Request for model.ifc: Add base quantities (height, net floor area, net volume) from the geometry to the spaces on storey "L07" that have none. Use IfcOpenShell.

First a look at what the model holds.

```python
import ifcopenshell
import ifcopenshell.util.element
import ifcopenshell.util.unit

model = ifcopenshell.open("model.ifc")
print(model.schema)
for unit_type in ("LENGTHUNIT", "AREAUNIT", "VOLUMEUNIT"):
    print(unit_type, ifcopenshell.util.unit.calculate_unit_scale(model, unit_type))
storey = next(s for s in model.by_type("IfcBuildingStorey") if s.Name == "L07")
spaces = [e for e in ifcopenshell.util.element.get_decomposition(storey) if e.is_a("IfcSpace")]
for e in sorted(spaces, key=lambda e: e.id()):
    print(e.id(), e.is_a(), e.Name, list(ifcopenshell.util.element.get_psets(e, qtos_only=True)), sep=" | ")
```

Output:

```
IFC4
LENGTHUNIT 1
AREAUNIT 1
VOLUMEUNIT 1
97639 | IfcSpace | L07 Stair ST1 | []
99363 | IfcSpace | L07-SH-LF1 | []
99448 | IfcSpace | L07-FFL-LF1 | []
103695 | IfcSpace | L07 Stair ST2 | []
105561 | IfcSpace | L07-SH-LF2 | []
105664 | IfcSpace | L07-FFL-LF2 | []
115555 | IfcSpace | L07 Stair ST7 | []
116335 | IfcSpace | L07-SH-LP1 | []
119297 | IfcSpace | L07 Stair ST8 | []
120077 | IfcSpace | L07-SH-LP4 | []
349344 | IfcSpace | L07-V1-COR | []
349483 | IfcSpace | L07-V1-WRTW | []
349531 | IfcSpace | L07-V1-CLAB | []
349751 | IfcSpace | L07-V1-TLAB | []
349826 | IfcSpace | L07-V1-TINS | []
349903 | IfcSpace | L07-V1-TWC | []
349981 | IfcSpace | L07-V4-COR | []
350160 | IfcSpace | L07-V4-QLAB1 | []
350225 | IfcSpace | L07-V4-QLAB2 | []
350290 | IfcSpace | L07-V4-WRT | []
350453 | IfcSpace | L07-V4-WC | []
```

```python
import ifcopenshell
import ifcopenshell.api.pset
import ifcopenshell.geom
import ifcopenshell.util.element
import ifcopenshell.util.shape
import ifcopenshell.util.unit

model = ifcopenshell.open("model.ifc")
unit_scale = ifcopenshell.util.unit.calculate_unit_scale(model)
area_scale = ifcopenshell.util.unit.calculate_unit_scale(model, "AREAUNIT")
volume_scale = ifcopenshell.util.unit.calculate_unit_scale(model, "VOLUMEUNIT")
settings = ifcopenshell.geom.settings()

storey = next(s for s in model.by_type("IfcBuildingStorey") if s.Name == "L07")
spaces = [e for e in ifcopenshell.util.element.get_decomposition(storey) if e.is_a("IfcSpace")]

for e in sorted(spaces, key=lambda e: e.id()):
    if ifcopenshell.util.element.get_psets(e, qtos_only=True, should_inherit=False):
        continue
    # Geometry comes back in metres, in the element's own axes.
    shape = ifcopenshell.geom.create_shape(settings, e)
    values = {
        "Height": ifcopenshell.util.shape.get_z(shape.geometry) / unit_scale,
        "NetFloorArea": ifcopenshell.util.shape.get_footprint_area(shape.geometry) / area_scale,
        "NetVolume": ifcopenshell.util.shape.get_volume(shape.geometry) / volume_scale,
    }
    qto = ifcopenshell.api.pset.add_qto(model, product=e, name="Qto_SpaceBaseQuantities")
    ifcopenshell.api.pset.edit_qto(model, qto=qto, properties=values)
    print(e.id(), {k: round(v, 3) for k, v in values.items()})

model.write("model_updated.ifc")
```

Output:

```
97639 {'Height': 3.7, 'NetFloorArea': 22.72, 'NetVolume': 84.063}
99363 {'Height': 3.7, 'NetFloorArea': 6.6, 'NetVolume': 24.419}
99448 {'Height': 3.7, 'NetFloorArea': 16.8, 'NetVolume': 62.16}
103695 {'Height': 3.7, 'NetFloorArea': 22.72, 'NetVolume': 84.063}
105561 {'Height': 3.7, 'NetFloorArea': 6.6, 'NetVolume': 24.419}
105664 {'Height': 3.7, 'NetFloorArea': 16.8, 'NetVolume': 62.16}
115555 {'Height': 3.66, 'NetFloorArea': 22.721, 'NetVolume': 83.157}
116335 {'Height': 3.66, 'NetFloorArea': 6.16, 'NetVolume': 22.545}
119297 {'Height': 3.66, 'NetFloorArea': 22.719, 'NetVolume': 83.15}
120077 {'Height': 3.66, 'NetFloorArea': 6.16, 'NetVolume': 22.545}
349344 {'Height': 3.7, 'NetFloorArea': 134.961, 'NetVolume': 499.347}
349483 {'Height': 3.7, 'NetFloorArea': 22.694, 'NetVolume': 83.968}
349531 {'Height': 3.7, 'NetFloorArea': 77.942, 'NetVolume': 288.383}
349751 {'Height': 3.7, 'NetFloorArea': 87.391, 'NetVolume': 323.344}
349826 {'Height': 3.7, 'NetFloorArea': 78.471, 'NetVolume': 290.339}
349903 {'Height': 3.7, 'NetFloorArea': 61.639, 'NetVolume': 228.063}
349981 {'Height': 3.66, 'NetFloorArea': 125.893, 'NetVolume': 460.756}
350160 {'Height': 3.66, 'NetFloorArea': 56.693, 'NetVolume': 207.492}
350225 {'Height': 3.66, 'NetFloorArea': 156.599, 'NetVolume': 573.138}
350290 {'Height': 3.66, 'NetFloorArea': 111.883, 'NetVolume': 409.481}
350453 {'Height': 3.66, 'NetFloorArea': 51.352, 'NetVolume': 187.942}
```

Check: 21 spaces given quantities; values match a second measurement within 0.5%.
